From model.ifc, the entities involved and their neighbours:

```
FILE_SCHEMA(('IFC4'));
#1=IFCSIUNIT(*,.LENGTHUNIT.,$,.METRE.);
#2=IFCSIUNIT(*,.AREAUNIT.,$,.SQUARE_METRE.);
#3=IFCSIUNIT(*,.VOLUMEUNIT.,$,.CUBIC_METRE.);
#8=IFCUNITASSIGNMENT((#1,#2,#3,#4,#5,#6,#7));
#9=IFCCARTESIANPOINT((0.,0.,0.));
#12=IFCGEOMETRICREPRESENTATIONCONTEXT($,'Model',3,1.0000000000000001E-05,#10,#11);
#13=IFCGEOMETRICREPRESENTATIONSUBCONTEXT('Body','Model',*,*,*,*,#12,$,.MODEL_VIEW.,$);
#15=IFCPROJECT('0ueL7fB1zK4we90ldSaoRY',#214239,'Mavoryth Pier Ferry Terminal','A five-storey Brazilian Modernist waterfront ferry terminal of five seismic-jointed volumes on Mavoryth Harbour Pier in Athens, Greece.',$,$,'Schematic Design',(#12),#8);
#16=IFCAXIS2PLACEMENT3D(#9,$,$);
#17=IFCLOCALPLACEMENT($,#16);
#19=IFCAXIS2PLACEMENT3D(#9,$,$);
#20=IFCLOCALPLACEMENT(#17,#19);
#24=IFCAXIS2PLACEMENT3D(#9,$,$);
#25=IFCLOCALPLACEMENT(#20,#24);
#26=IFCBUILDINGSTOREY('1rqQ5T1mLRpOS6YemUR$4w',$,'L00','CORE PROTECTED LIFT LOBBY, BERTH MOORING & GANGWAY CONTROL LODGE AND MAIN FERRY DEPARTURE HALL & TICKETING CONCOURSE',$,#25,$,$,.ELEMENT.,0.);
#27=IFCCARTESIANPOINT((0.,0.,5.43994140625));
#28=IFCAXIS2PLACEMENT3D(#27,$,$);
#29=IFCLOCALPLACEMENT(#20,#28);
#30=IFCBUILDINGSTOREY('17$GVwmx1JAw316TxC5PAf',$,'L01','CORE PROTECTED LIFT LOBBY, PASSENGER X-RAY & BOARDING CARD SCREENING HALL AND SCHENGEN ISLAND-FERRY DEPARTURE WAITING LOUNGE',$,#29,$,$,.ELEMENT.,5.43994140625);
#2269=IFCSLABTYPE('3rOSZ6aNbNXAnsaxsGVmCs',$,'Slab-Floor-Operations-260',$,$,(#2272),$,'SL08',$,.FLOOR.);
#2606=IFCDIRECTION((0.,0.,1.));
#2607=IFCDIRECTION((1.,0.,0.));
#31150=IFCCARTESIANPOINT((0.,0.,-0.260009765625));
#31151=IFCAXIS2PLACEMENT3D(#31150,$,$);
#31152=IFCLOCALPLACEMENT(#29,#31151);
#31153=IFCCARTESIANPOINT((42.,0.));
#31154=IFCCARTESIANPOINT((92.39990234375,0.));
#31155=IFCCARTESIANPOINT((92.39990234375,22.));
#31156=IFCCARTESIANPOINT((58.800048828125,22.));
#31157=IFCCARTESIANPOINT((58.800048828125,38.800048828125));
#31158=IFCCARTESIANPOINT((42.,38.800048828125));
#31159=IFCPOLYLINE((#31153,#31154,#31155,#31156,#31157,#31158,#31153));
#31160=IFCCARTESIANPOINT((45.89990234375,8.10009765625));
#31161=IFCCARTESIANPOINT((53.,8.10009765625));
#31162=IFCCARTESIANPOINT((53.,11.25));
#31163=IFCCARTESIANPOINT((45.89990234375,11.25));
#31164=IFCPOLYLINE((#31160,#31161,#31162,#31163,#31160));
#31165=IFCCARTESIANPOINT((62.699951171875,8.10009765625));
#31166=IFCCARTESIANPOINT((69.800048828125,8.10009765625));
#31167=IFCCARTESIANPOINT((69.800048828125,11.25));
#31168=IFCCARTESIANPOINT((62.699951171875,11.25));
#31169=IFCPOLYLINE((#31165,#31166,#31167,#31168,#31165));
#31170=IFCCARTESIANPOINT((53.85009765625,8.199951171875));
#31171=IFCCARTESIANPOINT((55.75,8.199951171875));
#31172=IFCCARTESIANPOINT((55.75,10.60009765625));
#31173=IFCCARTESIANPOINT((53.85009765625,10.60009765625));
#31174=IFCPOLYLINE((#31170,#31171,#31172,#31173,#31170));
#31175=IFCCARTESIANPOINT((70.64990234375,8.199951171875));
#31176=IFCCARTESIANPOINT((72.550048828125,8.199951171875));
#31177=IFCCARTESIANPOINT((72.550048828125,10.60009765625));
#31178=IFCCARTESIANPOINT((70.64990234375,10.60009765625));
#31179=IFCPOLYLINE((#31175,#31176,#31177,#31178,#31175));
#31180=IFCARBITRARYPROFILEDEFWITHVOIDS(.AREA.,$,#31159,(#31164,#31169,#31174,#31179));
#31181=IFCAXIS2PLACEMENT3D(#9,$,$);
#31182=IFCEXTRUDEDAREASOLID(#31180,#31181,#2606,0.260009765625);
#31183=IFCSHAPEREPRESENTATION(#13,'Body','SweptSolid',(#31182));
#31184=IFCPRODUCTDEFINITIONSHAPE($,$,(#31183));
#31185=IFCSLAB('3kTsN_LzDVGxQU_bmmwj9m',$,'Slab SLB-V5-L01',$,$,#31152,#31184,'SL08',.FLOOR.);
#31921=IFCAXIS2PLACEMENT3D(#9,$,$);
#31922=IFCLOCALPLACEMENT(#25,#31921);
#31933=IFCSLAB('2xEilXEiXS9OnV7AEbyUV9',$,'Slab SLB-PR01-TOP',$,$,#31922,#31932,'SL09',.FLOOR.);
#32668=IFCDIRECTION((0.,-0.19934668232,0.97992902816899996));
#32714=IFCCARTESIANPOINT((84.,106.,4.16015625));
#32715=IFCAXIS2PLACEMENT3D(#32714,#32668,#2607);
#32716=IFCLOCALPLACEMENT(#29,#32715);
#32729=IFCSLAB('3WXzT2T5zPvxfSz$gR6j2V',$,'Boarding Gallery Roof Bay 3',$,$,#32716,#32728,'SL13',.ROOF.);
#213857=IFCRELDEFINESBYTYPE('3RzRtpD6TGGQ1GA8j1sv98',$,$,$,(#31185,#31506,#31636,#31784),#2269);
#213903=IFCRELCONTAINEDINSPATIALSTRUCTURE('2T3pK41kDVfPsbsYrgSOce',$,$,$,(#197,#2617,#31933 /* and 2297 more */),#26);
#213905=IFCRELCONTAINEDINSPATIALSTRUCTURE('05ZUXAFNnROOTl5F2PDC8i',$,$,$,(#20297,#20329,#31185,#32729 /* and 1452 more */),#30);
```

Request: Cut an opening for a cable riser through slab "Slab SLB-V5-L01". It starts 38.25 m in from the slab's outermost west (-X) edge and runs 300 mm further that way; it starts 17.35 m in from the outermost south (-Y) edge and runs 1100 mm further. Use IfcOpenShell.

```python
import numpy as np
import ifcopenshell
import ifcopenshell.api.feature
import ifcopenshell.api.geometry
import ifcopenshell.api.root
import ifcopenshell.geom
import ifcopenshell.util.placement
import ifcopenshell.util.representation
import ifcopenshell.util.shape
import ifcopenshell.util.unit

model = ifcopenshell.open("model.ifc")
unit_scale = ifcopenshell.util.unit.calculate_unit_scale(model)
settings = ifcopenshell.geom.settings()


def volume(element):
    """Net volume in cubic metres, openings subtracted."""
    shape = ifcopenshell.geom.create_shape(settings, element)
    return ifcopenshell.util.shape.get_volume(shape.geometry)


slab = model.by_guid("3kTsN_LzDVGxQU_bmmwj9m")
before = volume(slab)

# Extent in the slab's own axes, in metres. The edges named are its -X and -Y sides.
slab_shape = ifcopenshell.geom.create_shape(settings, slab)
vertices = ifcopenshell.util.shape.get_vertices(slab_shape.geometry)
x_min, y_min, bottom = vertices.min(axis=0)
top = vertices[:, 2].max()

opening = ifcopenshell.api.root.create_entity(model, ifc_class="IfcOpeningElement", name="Cable riser opening", predefined_type="OPENING")
context = ifcopenshell.util.representation.get_context(model, "Model", "Body", "MODEL_VIEW")
width, depth = 0.3, 1.1
outline = [(0.0, 0.0), (width, 0.0), (width, depth), (0.0, depth), (0.0, 0.0)]
# Overshoot both faces by 50 mm so the cut is clean.
shape = ifcopenshell.api.geometry.add_slab_representation(
    model, context=context, depth=top - bottom + 0.1, polyline=outline
)
ifcopenshell.api.geometry.assign_representation(model, product=opening, representation=shape)

matrix = ifcopenshell.util.placement.get_local_placement(slab.ObjectPlacement)
matrix[:, 3] = matrix @ np.append(np.array([x_min + 38.25, y_min + 17.35, bottom - 0.05]) / unit_scale, 1.0)
ifcopenshell.api.geometry.edit_object_placement(model, product=opening, matrix=matrix, is_si=False)
ifcopenshell.api.feature.add_feature(model, feature=opening, element=slab)

after = volume(slab)

print(f"slab volume {before:.3f} -> {after:.3f} m3")

model.write("model-out.ifc")
```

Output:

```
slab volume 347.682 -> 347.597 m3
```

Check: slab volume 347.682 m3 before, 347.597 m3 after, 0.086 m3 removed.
